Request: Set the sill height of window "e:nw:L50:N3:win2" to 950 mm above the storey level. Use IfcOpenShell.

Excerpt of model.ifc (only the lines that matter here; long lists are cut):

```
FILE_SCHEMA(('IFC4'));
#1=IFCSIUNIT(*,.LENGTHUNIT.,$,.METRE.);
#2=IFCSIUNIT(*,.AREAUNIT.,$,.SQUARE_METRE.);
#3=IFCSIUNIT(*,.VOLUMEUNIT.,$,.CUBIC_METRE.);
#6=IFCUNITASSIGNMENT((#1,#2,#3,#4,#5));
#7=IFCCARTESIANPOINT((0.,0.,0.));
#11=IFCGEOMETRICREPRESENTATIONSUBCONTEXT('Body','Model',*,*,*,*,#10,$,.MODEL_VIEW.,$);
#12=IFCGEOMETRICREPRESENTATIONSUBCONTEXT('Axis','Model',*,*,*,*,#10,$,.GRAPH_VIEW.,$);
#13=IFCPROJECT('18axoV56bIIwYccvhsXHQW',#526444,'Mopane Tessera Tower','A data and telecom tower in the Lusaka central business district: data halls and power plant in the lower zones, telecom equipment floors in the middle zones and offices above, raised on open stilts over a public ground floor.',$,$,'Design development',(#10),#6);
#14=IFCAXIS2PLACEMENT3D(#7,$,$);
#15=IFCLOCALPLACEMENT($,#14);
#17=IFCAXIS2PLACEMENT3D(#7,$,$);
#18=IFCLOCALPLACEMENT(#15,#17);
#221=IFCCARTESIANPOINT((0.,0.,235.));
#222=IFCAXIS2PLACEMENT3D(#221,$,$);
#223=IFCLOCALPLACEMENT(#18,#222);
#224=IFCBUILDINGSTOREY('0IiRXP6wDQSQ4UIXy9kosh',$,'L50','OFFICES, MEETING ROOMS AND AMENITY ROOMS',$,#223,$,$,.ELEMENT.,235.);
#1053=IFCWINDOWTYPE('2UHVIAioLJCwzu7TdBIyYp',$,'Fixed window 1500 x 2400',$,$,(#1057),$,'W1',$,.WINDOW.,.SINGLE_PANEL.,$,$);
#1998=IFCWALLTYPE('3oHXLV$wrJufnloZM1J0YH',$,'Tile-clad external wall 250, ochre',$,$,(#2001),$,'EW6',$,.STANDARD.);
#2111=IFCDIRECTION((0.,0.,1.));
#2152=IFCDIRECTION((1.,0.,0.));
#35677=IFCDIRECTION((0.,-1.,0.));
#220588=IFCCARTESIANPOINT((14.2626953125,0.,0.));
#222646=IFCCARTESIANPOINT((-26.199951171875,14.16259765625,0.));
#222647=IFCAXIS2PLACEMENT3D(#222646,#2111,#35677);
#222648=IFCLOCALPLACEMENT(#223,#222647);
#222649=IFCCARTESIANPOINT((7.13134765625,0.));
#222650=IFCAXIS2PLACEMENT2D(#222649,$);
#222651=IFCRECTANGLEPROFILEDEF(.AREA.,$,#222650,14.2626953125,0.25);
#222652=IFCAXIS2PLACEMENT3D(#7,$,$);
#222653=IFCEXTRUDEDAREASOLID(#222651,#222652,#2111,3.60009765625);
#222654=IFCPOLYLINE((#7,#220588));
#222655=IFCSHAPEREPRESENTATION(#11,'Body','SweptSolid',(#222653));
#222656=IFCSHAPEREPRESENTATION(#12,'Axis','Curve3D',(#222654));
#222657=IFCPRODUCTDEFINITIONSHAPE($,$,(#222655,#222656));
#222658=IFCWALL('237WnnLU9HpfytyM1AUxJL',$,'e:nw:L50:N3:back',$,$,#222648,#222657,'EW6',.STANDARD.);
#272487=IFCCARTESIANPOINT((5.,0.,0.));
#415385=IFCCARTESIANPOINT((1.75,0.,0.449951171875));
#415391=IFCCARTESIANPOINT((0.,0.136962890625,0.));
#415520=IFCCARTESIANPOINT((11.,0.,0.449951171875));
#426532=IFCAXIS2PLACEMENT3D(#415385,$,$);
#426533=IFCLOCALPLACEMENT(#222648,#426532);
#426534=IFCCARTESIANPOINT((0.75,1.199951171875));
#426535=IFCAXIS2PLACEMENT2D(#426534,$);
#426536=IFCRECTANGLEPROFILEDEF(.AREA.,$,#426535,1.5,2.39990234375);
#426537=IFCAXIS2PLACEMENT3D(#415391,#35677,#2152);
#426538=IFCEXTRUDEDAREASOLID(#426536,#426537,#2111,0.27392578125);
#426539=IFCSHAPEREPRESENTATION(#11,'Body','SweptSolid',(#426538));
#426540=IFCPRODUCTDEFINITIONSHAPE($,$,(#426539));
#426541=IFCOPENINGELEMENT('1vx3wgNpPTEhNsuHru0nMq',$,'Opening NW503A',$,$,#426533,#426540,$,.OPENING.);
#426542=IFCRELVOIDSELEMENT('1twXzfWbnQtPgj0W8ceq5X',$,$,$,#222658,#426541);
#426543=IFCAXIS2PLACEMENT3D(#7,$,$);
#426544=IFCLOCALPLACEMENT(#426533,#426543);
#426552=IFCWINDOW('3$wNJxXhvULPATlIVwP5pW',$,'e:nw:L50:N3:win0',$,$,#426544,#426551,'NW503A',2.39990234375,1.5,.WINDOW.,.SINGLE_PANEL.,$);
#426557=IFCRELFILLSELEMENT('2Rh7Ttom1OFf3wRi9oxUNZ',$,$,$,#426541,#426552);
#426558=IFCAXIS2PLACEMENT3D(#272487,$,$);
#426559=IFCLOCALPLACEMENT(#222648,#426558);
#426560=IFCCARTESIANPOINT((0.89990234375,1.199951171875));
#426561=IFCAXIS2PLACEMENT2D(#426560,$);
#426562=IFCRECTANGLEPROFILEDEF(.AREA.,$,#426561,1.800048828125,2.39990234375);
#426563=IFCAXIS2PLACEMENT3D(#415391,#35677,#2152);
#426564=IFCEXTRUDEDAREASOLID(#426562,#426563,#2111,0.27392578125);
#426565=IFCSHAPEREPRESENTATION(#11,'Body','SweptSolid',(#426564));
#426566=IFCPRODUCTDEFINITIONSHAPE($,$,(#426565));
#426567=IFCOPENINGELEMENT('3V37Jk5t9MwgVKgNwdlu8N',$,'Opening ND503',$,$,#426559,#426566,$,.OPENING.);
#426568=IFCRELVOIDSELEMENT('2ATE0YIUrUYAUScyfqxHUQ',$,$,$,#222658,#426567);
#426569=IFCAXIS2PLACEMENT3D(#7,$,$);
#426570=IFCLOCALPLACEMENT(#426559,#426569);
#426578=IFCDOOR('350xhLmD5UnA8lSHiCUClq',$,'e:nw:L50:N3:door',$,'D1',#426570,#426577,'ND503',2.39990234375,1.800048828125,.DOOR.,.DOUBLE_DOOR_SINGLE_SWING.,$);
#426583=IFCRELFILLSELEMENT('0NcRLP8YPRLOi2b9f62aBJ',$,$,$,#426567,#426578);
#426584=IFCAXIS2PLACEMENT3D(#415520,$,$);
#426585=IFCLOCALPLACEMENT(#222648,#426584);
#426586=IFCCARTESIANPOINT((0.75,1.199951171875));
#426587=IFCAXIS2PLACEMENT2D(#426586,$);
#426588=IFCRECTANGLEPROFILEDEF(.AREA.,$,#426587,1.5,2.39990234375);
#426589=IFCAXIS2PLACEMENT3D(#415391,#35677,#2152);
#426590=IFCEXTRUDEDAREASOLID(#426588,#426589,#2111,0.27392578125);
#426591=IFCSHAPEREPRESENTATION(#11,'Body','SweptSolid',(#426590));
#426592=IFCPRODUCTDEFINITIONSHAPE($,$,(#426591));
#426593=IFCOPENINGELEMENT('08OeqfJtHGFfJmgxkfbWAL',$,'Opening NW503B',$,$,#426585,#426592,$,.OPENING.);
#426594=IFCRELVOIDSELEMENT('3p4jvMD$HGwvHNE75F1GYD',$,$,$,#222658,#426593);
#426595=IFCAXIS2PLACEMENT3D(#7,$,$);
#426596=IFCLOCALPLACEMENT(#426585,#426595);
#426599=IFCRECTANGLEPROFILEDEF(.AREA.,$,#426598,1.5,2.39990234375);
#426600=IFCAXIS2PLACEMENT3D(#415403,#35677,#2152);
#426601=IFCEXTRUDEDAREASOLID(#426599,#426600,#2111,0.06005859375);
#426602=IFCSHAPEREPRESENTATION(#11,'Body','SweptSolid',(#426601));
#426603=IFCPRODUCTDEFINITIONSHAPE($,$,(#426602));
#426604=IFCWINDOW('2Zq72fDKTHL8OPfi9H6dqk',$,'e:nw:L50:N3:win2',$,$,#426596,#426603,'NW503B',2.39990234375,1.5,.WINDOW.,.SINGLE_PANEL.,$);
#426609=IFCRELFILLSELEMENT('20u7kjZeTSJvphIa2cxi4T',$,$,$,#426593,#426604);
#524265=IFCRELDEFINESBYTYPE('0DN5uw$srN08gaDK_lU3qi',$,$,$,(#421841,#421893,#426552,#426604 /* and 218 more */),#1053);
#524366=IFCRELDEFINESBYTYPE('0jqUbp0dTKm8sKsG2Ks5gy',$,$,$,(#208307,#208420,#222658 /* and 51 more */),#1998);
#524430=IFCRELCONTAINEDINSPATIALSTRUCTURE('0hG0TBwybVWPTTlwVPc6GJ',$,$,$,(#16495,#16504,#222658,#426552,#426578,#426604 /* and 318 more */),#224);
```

```python
import numpy as np
import ifcopenshell
import ifcopenshell.api.geometry
import ifcopenshell.geom
import ifcopenshell.util.element
import ifcopenshell.util.placement
import ifcopenshell.util.shape
import ifcopenshell.util.unit

model = ifcopenshell.open("model.ifc")
unit_scale = ifcopenshell.util.unit.calculate_unit_scale(model)

window = model.by_id(426604)
opening = window.FillsVoids[0].RelatingOpeningElement
storey = ifcopenshell.util.element.get_container(window, ifc_class="IfcBuildingStorey")
level = ifcopenshell.util.placement.get_local_placement(storey.ObjectPlacement)[2, 3]

# The opening's origin need not be at the sill, so measure its lowest point.
shape = ifcopenshell.geom.create_shape(ifcopenshell.geom.settings(), opening)
bottom = ifcopenshell.util.shape.get_shape_bottom_elevation(shape, shape.geometry) / unit_scale
dz = level + 0.95 - bottom

shift = np.array([0.0, 0.0, dz])
# The window is placed relative to its opening, so it follows when the opening moves.
matrix = ifcopenshell.util.placement.get_local_placement(opening.ObjectPlacement)
matrix[:3, 3] += shift
ifcopenshell.api.geometry.edit_object_placement(
    model, product=opening, matrix=matrix, is_si=False, should_transform_children=True
)

print(f"moved by {dz * unit_scale:+.3f} m")

model.write("model_updated.ifc")
```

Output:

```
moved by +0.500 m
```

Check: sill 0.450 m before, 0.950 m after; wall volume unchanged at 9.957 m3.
